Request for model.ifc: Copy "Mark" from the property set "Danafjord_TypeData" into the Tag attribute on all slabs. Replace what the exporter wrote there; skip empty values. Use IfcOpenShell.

First a look at what the model holds.

```python
import ifcopenshell
import ifcopenshell.util.element

model = ifcopenshell.open("model.ifc")
print(model.schema)
slabs = model.by_type("IfcSlab")
print(len(slabs), "slabs")
for e in slabs[:8]:
    source = ifcopenshell.util.element.get_pset(e, "Danafjord_TypeData", "Mark")
    target = e.Tag
    print(e.id(), repr(source), repr(target), sep=" | ")
```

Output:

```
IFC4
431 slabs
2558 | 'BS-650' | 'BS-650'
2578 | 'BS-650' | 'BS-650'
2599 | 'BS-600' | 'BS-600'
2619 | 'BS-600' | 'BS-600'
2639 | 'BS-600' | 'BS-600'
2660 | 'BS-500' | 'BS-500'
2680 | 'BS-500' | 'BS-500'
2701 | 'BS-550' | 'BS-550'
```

```python
import ifcopenshell
import ifcopenshell.util.element

model = ifcopenshell.open("model.ifc")

count = 0
for e in model.by_type("IfcSlab"):
    value = ifcopenshell.util.element.get_pset(e, "Danafjord_TypeData", "Mark")
    current = e.Tag
    if not value or not value.strip() or current == value:
        continue
    e.Tag = value
    count += 1

print(count, "slabs updated")

model.write("model-out.ifc")
```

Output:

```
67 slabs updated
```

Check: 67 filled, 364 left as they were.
